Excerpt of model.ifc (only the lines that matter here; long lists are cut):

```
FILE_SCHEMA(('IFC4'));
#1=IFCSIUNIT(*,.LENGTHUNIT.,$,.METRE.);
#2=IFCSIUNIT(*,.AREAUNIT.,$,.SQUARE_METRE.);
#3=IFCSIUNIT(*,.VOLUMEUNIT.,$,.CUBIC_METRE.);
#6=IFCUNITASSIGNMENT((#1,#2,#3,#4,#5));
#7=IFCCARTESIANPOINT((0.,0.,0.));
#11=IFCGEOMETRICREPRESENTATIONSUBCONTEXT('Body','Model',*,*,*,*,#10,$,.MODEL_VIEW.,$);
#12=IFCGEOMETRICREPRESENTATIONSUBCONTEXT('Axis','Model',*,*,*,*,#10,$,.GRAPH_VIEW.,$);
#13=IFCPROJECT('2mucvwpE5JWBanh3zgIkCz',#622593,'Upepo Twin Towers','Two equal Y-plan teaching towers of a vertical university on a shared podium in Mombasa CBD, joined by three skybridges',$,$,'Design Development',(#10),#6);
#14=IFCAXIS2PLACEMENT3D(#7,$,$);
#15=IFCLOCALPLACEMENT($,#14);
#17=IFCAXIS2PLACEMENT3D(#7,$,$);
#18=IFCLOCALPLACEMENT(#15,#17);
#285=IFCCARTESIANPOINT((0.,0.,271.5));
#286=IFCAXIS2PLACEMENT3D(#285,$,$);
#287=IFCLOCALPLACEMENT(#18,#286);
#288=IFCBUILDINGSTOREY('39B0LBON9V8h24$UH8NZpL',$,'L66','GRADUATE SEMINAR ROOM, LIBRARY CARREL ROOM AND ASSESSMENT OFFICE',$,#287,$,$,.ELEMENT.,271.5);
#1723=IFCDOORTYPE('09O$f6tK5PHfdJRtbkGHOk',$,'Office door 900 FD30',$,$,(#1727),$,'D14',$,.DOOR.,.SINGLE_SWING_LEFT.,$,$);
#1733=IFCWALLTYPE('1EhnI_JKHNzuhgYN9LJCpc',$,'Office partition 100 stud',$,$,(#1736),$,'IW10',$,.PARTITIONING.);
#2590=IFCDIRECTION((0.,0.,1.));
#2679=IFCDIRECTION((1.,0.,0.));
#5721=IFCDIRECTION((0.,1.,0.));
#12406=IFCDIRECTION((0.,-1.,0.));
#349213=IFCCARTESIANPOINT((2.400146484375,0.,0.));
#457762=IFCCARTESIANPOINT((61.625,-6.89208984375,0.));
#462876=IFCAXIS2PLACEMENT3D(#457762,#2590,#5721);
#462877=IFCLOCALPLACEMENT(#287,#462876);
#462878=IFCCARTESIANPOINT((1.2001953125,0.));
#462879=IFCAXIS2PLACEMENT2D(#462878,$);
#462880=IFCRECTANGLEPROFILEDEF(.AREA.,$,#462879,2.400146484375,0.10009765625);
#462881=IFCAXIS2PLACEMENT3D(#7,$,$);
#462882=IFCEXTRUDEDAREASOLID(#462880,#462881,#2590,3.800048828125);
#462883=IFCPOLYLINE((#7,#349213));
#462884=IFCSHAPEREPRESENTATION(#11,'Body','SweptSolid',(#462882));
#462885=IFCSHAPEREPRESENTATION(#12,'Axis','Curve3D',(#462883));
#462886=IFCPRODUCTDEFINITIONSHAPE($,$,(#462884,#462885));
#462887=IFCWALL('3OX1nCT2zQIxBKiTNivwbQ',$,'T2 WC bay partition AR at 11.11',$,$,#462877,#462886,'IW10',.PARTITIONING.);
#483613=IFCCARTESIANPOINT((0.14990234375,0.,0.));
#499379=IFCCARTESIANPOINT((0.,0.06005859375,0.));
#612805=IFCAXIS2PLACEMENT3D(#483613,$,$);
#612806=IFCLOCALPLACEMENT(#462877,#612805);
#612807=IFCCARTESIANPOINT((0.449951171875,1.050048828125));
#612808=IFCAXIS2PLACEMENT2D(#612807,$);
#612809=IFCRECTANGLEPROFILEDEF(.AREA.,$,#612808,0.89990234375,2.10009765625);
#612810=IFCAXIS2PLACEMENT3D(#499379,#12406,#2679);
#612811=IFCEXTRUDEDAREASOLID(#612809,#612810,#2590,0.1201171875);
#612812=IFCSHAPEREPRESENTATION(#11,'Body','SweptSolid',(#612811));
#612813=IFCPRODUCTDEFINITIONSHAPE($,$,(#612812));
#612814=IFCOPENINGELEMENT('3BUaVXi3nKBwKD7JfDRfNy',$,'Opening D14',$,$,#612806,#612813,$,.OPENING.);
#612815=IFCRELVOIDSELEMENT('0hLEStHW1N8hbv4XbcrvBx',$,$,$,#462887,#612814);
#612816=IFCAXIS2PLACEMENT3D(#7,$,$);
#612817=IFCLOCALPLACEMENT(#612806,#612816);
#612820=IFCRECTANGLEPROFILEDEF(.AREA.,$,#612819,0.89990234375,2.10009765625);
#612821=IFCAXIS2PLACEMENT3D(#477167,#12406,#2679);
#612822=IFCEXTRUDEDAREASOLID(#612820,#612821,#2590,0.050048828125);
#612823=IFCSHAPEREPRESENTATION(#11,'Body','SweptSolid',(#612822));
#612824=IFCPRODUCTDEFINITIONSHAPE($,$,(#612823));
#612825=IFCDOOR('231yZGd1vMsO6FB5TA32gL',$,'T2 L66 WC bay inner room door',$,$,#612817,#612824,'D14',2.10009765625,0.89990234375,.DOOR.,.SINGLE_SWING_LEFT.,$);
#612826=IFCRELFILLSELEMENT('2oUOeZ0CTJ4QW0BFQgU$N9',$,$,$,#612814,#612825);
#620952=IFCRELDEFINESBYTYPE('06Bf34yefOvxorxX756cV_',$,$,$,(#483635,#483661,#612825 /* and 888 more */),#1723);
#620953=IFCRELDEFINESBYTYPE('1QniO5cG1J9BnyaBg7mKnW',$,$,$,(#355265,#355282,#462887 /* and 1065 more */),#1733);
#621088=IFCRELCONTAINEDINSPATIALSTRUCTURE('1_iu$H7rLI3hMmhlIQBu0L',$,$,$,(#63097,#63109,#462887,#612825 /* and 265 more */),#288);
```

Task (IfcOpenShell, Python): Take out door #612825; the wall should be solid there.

```python
import ifcopenshell
import ifcopenshell.api.feature
import ifcopenshell.api.root
import ifcopenshell.geom
import ifcopenshell.util.shape

model = ifcopenshell.open("model.ifc")
settings = ifcopenshell.geom.settings()


def volume(element):
    """Net volume in cubic metres, openings subtracted."""
    shape = ifcopenshell.geom.create_shape(settings, element)
    return ifcopenshell.util.shape.get_volume(shape.geometry)


door = model.by_id(612825)
opening = door.FillsVoids[0].RelatingOpeningElement
wall = opening.VoidsElements[0].RelatingBuildingElement
before = volume(wall)

ifcopenshell.api.root.remove_product(model, product=door)
ifcopenshell.api.feature.remove_feature(model, feature=opening)

after = volume(wall)

print(f"wall volume {before:.3f} -> {after:.3f} m3")

model.write("model_updated.ifc")
```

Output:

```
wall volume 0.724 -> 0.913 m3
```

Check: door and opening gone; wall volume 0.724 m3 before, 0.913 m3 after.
